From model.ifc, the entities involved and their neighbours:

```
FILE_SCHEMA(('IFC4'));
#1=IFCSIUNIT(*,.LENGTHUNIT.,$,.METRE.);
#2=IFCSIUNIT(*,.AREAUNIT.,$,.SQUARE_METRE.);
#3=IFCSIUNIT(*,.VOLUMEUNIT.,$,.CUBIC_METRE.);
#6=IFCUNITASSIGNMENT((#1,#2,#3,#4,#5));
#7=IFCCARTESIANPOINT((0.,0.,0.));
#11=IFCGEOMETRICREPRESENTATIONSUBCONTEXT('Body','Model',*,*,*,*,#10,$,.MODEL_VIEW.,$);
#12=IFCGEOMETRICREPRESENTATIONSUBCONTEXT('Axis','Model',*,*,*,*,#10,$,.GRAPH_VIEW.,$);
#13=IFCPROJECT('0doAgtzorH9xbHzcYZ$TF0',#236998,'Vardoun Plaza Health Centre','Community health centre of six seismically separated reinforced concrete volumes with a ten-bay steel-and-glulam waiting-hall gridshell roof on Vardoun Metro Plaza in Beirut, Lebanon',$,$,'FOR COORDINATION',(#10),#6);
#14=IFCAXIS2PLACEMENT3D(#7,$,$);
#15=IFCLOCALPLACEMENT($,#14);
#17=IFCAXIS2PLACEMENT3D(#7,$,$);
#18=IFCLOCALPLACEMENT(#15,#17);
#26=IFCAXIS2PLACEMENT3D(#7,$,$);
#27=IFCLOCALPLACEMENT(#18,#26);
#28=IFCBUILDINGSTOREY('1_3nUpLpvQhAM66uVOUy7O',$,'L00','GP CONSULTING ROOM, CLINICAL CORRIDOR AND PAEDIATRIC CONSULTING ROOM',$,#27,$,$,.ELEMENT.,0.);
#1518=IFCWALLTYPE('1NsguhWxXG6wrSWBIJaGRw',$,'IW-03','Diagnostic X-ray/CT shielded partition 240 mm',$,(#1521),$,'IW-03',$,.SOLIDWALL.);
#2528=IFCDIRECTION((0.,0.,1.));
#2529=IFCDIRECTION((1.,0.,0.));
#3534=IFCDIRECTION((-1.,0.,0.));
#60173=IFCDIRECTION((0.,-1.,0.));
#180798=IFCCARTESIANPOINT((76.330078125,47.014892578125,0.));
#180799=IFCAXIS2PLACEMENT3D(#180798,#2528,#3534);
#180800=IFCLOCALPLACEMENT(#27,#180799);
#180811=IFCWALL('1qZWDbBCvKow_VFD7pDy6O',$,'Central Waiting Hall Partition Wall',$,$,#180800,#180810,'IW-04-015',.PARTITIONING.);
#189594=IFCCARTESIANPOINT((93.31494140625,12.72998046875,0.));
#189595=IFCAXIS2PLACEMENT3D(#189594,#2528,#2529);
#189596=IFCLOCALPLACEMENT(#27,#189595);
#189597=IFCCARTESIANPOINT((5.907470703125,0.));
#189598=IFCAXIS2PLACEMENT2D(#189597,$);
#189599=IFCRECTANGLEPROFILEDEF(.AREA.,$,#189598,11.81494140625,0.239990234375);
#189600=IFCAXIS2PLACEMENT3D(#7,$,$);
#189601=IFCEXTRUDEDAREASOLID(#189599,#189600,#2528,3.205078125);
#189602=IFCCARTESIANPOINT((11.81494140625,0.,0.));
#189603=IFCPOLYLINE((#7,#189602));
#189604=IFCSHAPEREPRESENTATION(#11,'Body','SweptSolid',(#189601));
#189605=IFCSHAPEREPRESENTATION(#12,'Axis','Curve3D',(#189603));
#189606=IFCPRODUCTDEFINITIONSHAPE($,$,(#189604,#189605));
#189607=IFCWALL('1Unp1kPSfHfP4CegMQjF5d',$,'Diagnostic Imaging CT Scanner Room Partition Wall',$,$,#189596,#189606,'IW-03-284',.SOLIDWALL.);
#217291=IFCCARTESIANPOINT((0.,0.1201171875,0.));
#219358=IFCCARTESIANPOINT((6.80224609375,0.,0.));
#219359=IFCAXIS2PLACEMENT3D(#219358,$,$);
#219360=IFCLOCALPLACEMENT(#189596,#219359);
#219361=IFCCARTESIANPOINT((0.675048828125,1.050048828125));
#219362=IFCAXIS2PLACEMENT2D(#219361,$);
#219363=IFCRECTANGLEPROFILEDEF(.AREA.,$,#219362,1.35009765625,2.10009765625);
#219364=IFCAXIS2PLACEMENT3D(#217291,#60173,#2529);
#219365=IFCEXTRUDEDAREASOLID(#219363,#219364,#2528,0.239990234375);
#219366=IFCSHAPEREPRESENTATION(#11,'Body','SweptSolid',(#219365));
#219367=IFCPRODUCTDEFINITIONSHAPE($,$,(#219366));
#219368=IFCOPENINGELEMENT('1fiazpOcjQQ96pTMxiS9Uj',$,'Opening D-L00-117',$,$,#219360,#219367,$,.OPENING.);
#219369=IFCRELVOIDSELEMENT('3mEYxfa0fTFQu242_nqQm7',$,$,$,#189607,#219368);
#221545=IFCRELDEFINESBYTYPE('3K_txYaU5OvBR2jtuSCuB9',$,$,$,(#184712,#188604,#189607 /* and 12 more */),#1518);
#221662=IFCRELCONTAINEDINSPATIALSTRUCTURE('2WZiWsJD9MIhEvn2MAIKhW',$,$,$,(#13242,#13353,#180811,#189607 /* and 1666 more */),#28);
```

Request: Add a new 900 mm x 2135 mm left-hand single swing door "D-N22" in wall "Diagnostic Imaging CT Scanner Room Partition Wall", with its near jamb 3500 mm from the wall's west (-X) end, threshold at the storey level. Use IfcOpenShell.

```python
import numpy as np
import ifcopenshell
import ifcopenshell.api.feature
import ifcopenshell.api.geometry
import ifcopenshell.api.root
import ifcopenshell.api.spatial
import ifcopenshell.geom
import ifcopenshell.util.element
import ifcopenshell.util.placement
import ifcopenshell.util.representation
import ifcopenshell.util.shape
import ifcopenshell.util.unit

model = ifcopenshell.open("model.ifc")
unit_scale = ifcopenshell.util.unit.calculate_unit_scale(model)
settings = ifcopenshell.geom.settings()


def volume(element):
    """Net volume in cubic metres, openings subtracted."""
    shape = ifcopenshell.geom.create_shape(settings, element)
    return ifcopenshell.util.shape.get_volume(shape.geometry)


wall = model.by_guid("1Unp1kPSfHfP4CegMQjF5d")
storey = ifcopenshell.util.element.get_container(wall, ifc_class="IfcBuildingStorey")
context = ifcopenshell.util.representation.get_context(model, "Model", "Body", "MODEL_VIEW")
before = volume(wall)

width, height, from_end, sill = 0.9, 2.135, 3.5, 0.0  # metres

# The wall runs along its own X axis, and the end named is its -X end.
wall_shape = ifcopenshell.geom.create_shape(settings, wall)
x, y, z = ifcopenshell.util.shape.get_vertices(wall_shape.geometry).T
start = x.min() + from_end
face, thickness = float(y.min()), float(y.max() - y.min())
wall_matrix = ifcopenshell.util.placement.get_local_placement(wall.ObjectPlacement)
level = ifcopenshell.util.placement.get_local_placement(storey.ObjectPlacement)[2, 3]


def in_wall(x, y):
    """Placement at x, y metres in the wall's axes, at sill height."""
    matrix = wall_matrix.copy()
    matrix[:, 3] = wall_matrix @ np.array([x / unit_scale, y / unit_scale, 0.0, 1.0])
    matrix[2, 3] = level + sill / unit_scale
    return matrix


# Opening: a box that overshoots both wall faces by 50 mm.
opening = ifcopenshell.api.root.create_entity(model, ifc_class="IfcOpeningElement", predefined_type="OPENING")
box = ifcopenshell.api.geometry.add_wall_representation(
    model, context=context, length=width, height=height, thickness=thickness + 0.1
)
ifcopenshell.api.geometry.assign_representation(model, product=opening, representation=box)
ifcopenshell.api.geometry.edit_object_placement(model, product=opening, matrix=in_wall(start, face - 0.05), is_si=False)
ifcopenshell.api.feature.add_feature(model, feature=opening, element=wall)

door = ifcopenshell.api.root.create_entity(model, ifc_class="IfcDoor", name="D-N22", predefined_type="DOOR")
door.OverallWidth, door.OverallHeight = width / unit_scale, height / unit_scale
door.OperationType = "SINGLE_SWING_LEFT"
body = ifcopenshell.api.geometry.add_door_representation(
    model,
    context=context,
    overall_width=door.OverallWidth,
    overall_height=door.OverallHeight,
    operation_type="SINGLE_SWING_LEFT",
    lining_properties={"LiningDepth": thickness / unit_scale, "ThresholdDepth": thickness / unit_scale},
)
ifcopenshell.api.geometry.assign_representation(model, product=door, representation=body)
ifcopenshell.api.spatial.assign_container(model, products=[door], relating_structure=storey)
ifcopenshell.api.feature.add_filling(model, opening=opening, element=door)

# The lining spans the wall, so the door starts at the wall face.
ifcopenshell.api.geometry.edit_object_placement(model, product=door, matrix=in_wall(start, face), is_si=False)

after = volume(wall)

print(f"wall volume {before:.3f} -> {after:.3f} m3")

model.write("model_v2.ifc")
```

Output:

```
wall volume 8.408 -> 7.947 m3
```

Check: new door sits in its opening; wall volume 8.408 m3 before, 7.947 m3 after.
